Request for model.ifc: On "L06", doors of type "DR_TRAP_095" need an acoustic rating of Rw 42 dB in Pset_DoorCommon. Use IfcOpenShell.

First a look at what the model holds.

```python
import ifcopenshell
import ifcopenshell.util.element

model = ifcopenshell.open("model.ifc")
print(model.schema)
storey = next(s for s in model.by_type("IfcBuildingStorey") if s.Name == "L06")
doors = [e for e in ifcopenshell.util.element.get_decomposition(storey) if e.is_a("IfcDoor")]
seen = {}
for e in doors:
    element_type = ifcopenshell.util.element.get_type(e)
    key = (element_type.Name if element_type != e and element_type else None, ifcopenshell.util.element.get_pset(e, "Pset_DoorCommon", "AcousticRating"))
    seen[key] = seen.get(key, 0) + 1
for (name, value), count in sorted(seen.items(), key=str):
    print(count, "x", name, "|", value)
```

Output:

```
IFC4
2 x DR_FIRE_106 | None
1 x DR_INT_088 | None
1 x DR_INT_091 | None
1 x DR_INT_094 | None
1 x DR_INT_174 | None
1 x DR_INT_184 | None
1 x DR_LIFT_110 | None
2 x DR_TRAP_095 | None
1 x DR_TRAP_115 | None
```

```python
import ifcopenshell
import ifcopenshell.api.pset
import ifcopenshell.util.element

model = ifcopenshell.open("model.ifc")

storey = next(s for s in model.by_type("IfcBuildingStorey") if s.Name == "L06")
doors = [e for e in ifcopenshell.util.element.get_decomposition(storey) if e.is_a("IfcDoor")]

count = 0
for e in doors:
    element_type = ifcopenshell.util.element.get_type(e)
    if element_type in (None, e) or element_type.Name != "DR_TRAP_095":
        continue
    # add_pset returns the element's existing set when there is one.
    pset = ifcopenshell.api.pset.add_pset(model, product=e, name="Pset_DoorCommon")
    ifcopenshell.api.pset.edit_pset(model, pset=pset, properties={"AcousticRating": "Rw 42 dB"})
    count += 1

print(count, "doors updated")

model.write("model_updated.ifc")
```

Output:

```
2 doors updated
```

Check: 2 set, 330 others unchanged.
